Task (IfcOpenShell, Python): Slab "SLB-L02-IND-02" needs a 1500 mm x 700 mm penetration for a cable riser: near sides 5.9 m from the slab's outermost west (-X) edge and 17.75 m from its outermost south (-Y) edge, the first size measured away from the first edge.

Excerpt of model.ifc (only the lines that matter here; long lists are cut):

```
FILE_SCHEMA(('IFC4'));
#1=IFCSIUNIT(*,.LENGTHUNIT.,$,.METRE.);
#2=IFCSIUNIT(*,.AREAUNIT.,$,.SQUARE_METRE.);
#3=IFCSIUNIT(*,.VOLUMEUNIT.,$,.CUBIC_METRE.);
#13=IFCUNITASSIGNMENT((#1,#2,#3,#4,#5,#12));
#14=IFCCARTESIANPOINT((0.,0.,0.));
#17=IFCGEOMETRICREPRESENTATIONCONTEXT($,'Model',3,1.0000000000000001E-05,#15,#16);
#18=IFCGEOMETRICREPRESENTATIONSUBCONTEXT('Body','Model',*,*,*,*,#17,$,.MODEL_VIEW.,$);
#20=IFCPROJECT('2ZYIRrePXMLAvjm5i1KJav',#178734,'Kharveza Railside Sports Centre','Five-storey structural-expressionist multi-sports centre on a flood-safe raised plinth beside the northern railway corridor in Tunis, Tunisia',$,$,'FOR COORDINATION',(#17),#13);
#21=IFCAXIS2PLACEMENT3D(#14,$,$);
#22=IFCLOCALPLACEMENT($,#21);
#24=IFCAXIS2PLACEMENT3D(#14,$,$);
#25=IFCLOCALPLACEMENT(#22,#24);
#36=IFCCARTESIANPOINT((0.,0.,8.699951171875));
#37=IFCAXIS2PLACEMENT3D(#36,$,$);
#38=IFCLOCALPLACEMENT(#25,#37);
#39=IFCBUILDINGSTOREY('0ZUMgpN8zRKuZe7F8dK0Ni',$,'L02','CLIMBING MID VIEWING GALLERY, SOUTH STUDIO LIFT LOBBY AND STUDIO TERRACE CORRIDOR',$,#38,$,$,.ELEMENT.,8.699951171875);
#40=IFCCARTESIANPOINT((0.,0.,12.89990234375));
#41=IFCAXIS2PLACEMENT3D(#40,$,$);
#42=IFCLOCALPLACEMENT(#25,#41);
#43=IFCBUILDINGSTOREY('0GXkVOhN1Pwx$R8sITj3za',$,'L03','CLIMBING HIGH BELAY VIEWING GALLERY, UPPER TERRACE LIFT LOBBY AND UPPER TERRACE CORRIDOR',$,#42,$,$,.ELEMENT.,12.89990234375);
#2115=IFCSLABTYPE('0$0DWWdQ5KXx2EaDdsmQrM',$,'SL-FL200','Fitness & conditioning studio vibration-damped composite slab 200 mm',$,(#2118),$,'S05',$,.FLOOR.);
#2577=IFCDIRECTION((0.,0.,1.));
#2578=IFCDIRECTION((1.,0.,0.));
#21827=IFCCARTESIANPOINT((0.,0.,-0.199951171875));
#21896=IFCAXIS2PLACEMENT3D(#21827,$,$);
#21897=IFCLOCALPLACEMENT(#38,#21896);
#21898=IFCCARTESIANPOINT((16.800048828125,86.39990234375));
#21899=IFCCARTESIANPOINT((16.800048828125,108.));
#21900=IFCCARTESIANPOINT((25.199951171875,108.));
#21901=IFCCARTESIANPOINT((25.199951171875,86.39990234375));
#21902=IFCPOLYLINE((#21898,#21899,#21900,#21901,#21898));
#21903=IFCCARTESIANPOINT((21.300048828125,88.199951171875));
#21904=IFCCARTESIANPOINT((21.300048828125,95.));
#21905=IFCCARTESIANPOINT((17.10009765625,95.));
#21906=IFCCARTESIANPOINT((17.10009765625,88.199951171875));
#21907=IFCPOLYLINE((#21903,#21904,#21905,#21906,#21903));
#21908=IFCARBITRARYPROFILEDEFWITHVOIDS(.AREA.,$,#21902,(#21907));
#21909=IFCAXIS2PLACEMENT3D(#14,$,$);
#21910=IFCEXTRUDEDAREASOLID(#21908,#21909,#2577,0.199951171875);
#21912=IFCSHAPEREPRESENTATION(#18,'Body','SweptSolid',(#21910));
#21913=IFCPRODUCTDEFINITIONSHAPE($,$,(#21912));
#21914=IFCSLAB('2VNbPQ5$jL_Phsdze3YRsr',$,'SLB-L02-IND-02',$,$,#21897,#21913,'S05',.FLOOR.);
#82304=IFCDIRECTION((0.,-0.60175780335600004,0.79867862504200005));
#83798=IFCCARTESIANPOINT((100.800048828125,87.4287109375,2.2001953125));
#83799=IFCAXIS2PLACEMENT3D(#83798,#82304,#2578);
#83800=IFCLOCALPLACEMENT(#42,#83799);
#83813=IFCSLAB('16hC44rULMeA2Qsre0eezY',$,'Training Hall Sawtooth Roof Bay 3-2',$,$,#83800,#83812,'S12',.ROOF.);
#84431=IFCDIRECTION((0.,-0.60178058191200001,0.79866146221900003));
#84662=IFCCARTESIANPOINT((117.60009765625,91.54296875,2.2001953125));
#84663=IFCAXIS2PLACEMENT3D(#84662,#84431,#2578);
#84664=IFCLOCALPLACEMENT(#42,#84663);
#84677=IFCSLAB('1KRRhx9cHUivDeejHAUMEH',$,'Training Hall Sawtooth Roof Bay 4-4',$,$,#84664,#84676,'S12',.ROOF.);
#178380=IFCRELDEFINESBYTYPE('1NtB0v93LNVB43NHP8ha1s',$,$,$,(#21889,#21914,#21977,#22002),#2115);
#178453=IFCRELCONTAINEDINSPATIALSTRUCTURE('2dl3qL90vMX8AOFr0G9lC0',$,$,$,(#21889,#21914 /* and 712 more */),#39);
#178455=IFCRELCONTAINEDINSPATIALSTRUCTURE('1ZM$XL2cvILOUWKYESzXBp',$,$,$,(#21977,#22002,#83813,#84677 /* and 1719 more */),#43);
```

```python
import numpy as np
import ifcopenshell
import ifcopenshell.api.feature
import ifcopenshell.api.geometry
import ifcopenshell.api.root
import ifcopenshell.geom
import ifcopenshell.util.placement
import ifcopenshell.util.representation
import ifcopenshell.util.shape
import ifcopenshell.util.unit

model = ifcopenshell.open("model.ifc")
unit_scale = ifcopenshell.util.unit.calculate_unit_scale(model)
settings = ifcopenshell.geom.settings()


def volume(element):
    """Net volume in cubic metres, openings subtracted."""
    shape = ifcopenshell.geom.create_shape(settings, element)
    return ifcopenshell.util.shape.get_volume(shape.geometry)


slab = model.by_guid("2VNbPQ5$jL_Phsdze3YRsr")
before = volume(slab)

# Extent in the slab's own axes, in metres. The edges named are its -X and -Y sides.
slab_shape = ifcopenshell.geom.create_shape(settings, slab)
vertices = ifcopenshell.util.shape.get_vertices(slab_shape.geometry)
x_min, y_min, bottom = vertices.min(axis=0)
top = vertices[:, 2].max()

opening = ifcopenshell.api.root.create_entity(model, ifc_class="IfcOpeningElement", name="Cable riser opening", predefined_type="OPENING")
context = ifcopenshell.util.representation.get_context(model, "Model", "Body", "MODEL_VIEW")
width, depth = 1.5, 0.7
outline = [(0.0, 0.0), (width, 0.0), (width, depth), (0.0, depth), (0.0, 0.0)]
# Overshoot both faces by 50 mm so the cut is clean.
shape = ifcopenshell.api.geometry.add_slab_representation(
    model, context=context, depth=top - bottom + 0.1, polyline=outline
)
ifcopenshell.api.geometry.assign_representation(model, product=opening, representation=shape)

matrix = ifcopenshell.util.placement.get_local_placement(slab.ObjectPlacement)
matrix[:, 3] = matrix @ np.append(np.array([x_min + 5.9, y_min + 17.75, bottom - 0.05]) / unit_scale, 1.0)
ifcopenshell.api.geometry.edit_object_placement(model, product=opening, matrix=matrix, is_si=False)
ifcopenshell.api.feature.add_feature(model, feature=opening, element=slab)

after = volume(slab)

print(f"slab volume {before:.3f} -> {after:.3f} m3")

model.write("model_updated.ifc")
```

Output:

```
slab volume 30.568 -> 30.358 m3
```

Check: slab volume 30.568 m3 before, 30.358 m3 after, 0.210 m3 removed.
